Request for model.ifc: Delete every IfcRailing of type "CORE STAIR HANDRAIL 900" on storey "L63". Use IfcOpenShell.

First a look at what the model holds.

```python
import ifcopenshell
import ifcopenshell.util.element

model = ifcopenshell.open("model.ifc")
print(model.schema)
storey = next(s for s in model.by_type("IfcBuildingStorey") if s.Name == "L63")
railings = [e for e in ifcopenshell.util.element.get_decomposition(storey) if e.is_a("IfcRailing")]
seen = {}
for e in railings:
    element_type = ifcopenshell.util.element.get_type(e)
    name = element_type.Name if element_type not in (None, e) else None
    seen[name] = seen.get(name, 0) + 1
for name, count in sorted(seen.items(), key=str):
    print(count, "x", name)
```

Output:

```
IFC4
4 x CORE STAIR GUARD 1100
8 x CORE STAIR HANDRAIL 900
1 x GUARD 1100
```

```python
import ifcopenshell
import ifcopenshell.api.root
import ifcopenshell.util.element

model = ifcopenshell.open("model.ifc")

storey = next(s for s in model.by_type("IfcBuildingStorey") if s.Name == "L63")
railings = [e for e in ifcopenshell.util.element.get_decomposition(storey) if e.is_a("IfcRailing")]
targets = [e for e in railings if (t := ifcopenshell.util.element.get_type(e)) not in (None, e) and t.Name == "CORE STAIR HANDRAIL 900"]

for e in targets:
    ifcopenshell.api.root.remove_product(model, product=e)
print(len(targets), "removed")

model.write("model_v2.ifc")
```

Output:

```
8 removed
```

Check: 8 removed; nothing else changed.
